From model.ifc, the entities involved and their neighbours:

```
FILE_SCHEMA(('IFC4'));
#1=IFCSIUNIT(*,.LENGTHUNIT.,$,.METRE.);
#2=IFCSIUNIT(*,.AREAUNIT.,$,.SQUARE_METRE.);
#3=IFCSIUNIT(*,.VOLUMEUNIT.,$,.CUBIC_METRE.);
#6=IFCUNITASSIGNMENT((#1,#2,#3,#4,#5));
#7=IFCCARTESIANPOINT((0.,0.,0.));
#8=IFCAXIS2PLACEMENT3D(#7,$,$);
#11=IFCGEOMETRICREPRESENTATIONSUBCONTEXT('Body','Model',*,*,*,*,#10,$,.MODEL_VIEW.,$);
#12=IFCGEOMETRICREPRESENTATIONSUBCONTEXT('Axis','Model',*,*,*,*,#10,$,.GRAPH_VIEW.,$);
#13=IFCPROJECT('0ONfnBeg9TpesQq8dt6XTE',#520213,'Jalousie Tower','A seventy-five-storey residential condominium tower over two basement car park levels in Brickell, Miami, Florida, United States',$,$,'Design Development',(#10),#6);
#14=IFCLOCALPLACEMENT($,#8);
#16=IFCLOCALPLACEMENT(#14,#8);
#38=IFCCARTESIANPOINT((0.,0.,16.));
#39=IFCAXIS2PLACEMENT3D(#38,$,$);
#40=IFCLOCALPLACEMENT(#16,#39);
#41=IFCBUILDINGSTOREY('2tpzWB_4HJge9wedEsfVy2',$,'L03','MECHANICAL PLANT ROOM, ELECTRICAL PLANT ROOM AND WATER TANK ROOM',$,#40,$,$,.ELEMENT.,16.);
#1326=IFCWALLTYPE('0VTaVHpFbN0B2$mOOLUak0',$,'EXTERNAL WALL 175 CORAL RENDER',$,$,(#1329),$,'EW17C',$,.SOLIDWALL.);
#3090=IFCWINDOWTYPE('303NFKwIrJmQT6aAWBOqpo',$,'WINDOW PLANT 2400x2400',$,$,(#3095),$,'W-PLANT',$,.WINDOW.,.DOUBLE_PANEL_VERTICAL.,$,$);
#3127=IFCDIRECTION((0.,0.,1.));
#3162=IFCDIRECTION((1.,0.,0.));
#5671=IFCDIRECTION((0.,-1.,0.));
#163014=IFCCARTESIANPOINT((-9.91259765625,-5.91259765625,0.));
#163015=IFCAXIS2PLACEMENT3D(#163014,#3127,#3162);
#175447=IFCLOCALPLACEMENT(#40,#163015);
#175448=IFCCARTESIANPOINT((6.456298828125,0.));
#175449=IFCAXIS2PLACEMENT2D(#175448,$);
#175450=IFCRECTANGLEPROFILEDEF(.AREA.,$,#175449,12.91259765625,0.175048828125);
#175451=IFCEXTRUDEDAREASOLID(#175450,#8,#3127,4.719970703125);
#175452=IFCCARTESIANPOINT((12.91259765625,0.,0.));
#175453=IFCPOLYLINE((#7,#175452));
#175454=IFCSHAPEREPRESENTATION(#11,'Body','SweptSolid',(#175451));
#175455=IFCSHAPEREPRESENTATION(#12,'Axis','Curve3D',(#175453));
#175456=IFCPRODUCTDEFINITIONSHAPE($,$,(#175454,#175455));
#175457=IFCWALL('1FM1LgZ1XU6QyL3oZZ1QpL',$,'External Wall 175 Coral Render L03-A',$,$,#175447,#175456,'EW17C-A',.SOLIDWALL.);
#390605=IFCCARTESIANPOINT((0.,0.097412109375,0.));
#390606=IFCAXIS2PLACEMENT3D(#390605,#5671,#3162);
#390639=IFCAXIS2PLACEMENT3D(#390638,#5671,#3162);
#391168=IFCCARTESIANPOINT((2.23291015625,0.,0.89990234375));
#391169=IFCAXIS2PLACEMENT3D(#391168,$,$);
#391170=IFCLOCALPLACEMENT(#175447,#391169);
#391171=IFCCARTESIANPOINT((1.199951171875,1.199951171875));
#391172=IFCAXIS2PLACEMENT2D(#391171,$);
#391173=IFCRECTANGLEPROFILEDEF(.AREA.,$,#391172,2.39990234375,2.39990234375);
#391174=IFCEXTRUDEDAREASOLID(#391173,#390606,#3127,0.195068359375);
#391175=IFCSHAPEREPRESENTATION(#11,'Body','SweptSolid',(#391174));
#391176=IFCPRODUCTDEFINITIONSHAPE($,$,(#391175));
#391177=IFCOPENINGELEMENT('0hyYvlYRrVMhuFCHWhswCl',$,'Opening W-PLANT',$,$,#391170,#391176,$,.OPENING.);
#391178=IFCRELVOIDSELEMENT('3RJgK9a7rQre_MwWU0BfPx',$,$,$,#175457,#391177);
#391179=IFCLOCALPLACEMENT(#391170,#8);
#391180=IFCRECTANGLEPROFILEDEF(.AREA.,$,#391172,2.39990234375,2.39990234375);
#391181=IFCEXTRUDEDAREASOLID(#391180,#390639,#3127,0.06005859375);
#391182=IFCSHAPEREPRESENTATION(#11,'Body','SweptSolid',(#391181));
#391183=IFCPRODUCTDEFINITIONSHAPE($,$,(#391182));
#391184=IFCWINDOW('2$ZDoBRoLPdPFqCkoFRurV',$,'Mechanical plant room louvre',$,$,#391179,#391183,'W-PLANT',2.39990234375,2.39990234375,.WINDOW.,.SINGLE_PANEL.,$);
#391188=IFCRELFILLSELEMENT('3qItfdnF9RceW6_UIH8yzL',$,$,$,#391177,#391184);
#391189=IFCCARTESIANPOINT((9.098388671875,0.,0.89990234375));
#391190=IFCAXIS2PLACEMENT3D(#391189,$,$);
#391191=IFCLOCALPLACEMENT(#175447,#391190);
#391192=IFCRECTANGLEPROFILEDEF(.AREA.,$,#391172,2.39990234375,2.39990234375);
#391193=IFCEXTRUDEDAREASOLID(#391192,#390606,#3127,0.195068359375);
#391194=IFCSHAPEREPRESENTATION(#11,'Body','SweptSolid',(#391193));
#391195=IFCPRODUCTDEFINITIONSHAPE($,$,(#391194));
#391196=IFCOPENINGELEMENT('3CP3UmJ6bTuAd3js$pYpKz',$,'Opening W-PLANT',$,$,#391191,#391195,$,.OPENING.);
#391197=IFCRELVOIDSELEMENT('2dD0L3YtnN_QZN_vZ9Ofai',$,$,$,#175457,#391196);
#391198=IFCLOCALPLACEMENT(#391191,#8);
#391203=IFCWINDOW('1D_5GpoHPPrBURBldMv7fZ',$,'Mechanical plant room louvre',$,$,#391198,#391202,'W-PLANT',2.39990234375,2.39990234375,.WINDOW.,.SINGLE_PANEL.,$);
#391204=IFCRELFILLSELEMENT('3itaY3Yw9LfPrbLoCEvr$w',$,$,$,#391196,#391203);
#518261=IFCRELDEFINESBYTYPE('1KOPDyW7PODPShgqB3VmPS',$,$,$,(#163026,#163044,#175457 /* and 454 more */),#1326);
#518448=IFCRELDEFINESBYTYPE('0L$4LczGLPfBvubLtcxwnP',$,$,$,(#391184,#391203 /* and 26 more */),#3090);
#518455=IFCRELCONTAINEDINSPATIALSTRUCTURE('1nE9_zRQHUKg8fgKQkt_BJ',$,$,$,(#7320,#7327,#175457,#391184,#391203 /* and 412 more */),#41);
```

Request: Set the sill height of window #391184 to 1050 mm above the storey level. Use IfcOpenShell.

```python
import numpy as np
import ifcopenshell
import ifcopenshell.api.geometry
import ifcopenshell.geom
import ifcopenshell.util.element
import ifcopenshell.util.placement
import ifcopenshell.util.shape
import ifcopenshell.util.unit

model = ifcopenshell.open("model.ifc")
unit_scale = ifcopenshell.util.unit.calculate_unit_scale(model)

window = model.by_id(391184)
opening = window.FillsVoids[0].RelatingOpeningElement
storey = ifcopenshell.util.element.get_container(window, ifc_class="IfcBuildingStorey")
level = ifcopenshell.util.placement.get_local_placement(storey.ObjectPlacement)[2, 3]

# The opening's origin need not be at the sill, so measure its lowest point.
shape = ifcopenshell.geom.create_shape(ifcopenshell.geom.settings(), opening)
bottom = ifcopenshell.util.shape.get_shape_bottom_elevation(shape, shape.geometry) / unit_scale
dz = level + 1.05 / unit_scale - bottom

shift = np.array([0.0, 0.0, dz])
# The window is placed relative to its opening, so it follows when the opening moves.
matrix = ifcopenshell.util.placement.get_local_placement(opening.ObjectPlacement)
matrix[:3, 3] += shift
ifcopenshell.api.geometry.edit_object_placement(
    model, product=opening, matrix=matrix, is_si=False, should_transform_children=True
)

print(f"moved by {dz * unit_scale:+.3f} m")

model.write("model-out.ifc")
```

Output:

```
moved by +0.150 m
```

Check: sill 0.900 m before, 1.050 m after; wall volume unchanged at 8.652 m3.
